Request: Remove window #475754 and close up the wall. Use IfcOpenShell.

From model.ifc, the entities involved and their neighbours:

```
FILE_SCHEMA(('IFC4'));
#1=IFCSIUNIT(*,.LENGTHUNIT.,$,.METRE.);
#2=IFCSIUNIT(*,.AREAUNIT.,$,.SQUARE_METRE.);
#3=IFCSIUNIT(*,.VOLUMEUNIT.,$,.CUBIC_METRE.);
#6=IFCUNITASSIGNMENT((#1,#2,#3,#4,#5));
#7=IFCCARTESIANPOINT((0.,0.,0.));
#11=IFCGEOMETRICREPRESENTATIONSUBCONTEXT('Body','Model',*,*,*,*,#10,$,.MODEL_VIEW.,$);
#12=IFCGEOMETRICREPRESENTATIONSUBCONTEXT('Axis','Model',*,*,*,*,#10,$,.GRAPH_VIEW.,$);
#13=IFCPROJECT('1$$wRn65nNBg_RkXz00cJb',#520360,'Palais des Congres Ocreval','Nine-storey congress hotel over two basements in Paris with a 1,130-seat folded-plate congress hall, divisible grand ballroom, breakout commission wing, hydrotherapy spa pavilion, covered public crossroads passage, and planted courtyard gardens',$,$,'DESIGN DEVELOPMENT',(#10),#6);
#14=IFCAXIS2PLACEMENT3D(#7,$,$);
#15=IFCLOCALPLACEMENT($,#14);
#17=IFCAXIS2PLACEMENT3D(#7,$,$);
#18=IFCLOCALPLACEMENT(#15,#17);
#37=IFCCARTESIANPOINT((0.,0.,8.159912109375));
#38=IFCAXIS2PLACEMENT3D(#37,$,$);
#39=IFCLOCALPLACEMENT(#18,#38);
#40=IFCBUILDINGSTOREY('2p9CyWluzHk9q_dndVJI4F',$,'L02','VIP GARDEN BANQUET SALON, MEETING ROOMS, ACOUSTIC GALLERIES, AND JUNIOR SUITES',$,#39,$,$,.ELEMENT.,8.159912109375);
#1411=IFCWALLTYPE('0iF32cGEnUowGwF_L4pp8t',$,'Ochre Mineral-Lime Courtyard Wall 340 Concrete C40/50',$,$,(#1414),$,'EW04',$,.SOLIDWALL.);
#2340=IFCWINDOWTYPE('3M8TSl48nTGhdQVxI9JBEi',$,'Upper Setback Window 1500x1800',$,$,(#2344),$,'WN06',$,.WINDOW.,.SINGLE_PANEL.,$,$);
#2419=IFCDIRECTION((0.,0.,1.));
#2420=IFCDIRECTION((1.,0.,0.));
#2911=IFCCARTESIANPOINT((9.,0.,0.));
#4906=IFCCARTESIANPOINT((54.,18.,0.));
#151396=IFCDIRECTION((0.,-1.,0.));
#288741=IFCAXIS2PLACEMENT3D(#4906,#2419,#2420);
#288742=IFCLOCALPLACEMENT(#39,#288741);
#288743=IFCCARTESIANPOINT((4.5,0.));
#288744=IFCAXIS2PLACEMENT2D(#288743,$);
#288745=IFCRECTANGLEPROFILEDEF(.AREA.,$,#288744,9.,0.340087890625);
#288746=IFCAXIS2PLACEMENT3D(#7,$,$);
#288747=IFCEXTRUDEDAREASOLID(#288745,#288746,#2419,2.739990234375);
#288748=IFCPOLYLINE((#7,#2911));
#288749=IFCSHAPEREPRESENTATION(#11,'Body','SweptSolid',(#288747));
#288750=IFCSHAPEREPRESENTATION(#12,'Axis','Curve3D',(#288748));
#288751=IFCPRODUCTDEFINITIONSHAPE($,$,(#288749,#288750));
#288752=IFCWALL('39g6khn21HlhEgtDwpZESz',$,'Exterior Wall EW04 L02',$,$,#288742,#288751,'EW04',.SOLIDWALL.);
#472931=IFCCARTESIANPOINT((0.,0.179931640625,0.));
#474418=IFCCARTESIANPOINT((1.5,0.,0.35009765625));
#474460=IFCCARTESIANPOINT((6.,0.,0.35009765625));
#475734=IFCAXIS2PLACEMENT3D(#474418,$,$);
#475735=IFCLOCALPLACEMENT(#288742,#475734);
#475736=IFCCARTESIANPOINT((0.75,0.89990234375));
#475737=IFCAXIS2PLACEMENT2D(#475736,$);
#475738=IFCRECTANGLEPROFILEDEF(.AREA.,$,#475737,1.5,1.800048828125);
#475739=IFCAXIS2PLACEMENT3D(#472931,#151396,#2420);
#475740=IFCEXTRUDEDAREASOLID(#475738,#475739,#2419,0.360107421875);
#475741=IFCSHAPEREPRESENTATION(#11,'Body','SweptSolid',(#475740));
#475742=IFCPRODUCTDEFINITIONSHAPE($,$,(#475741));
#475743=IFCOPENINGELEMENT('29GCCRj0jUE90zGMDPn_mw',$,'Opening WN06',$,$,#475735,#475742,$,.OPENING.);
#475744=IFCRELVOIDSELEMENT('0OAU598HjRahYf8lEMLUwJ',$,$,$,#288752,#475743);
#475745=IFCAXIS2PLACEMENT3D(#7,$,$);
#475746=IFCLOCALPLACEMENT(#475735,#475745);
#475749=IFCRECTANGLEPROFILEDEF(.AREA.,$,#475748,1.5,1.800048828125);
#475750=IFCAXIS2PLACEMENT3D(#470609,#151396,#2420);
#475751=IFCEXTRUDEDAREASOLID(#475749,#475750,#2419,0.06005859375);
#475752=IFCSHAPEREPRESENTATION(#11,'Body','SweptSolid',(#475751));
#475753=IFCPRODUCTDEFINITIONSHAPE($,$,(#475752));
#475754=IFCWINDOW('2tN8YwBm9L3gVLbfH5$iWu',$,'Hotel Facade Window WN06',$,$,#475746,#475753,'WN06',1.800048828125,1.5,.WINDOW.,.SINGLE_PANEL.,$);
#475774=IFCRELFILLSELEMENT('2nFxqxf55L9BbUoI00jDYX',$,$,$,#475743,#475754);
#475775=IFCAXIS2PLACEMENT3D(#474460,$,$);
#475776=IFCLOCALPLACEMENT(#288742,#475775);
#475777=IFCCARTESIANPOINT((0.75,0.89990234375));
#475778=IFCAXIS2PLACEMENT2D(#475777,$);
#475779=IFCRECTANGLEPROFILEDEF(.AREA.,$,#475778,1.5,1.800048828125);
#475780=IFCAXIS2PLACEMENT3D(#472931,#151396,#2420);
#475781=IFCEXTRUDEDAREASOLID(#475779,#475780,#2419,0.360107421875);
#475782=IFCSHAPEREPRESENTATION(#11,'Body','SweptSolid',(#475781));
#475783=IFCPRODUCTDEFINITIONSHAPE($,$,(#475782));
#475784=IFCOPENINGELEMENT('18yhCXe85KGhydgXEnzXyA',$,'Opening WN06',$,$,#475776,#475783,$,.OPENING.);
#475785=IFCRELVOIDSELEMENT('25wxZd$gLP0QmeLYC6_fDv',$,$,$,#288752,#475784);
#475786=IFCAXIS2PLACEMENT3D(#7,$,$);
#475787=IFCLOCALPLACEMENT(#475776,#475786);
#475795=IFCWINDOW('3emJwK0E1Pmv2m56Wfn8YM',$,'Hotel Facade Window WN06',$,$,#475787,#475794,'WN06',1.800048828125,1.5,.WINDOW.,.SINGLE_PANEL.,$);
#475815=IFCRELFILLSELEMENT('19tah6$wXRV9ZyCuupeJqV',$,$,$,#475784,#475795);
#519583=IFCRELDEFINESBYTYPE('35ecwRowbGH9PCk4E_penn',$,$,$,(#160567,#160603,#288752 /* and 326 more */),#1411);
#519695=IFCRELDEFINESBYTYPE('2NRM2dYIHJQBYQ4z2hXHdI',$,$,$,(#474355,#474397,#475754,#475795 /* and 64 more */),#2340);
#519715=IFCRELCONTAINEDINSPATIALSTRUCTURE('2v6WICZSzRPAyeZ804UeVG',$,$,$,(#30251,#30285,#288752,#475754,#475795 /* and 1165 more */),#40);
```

```python
import ifcopenshell
import ifcopenshell.api.feature
import ifcopenshell.api.root
import ifcopenshell.geom
import ifcopenshell.util.shape

model = ifcopenshell.open("model.ifc")
settings = ifcopenshell.geom.settings()


def volume(element):
    """Net volume in cubic metres, openings subtracted."""
    shape = ifcopenshell.geom.create_shape(settings, element)
    return ifcopenshell.util.shape.get_volume(shape.geometry)


window = model.by_id(475754)
opening = window.FillsVoids[0].RelatingOpeningElement
wall = opening.VoidsElements[0].RelatingBuildingElement
before = volume(wall)

ifcopenshell.api.root.remove_product(model, product=window)
ifcopenshell.api.feature.remove_feature(model, feature=opening)

after = volume(wall)

print(f"wall volume {before:.3f} -> {after:.3f} m3")

model.write("model_edited.ifc")
```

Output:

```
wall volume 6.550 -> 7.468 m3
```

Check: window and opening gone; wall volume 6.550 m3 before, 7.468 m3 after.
